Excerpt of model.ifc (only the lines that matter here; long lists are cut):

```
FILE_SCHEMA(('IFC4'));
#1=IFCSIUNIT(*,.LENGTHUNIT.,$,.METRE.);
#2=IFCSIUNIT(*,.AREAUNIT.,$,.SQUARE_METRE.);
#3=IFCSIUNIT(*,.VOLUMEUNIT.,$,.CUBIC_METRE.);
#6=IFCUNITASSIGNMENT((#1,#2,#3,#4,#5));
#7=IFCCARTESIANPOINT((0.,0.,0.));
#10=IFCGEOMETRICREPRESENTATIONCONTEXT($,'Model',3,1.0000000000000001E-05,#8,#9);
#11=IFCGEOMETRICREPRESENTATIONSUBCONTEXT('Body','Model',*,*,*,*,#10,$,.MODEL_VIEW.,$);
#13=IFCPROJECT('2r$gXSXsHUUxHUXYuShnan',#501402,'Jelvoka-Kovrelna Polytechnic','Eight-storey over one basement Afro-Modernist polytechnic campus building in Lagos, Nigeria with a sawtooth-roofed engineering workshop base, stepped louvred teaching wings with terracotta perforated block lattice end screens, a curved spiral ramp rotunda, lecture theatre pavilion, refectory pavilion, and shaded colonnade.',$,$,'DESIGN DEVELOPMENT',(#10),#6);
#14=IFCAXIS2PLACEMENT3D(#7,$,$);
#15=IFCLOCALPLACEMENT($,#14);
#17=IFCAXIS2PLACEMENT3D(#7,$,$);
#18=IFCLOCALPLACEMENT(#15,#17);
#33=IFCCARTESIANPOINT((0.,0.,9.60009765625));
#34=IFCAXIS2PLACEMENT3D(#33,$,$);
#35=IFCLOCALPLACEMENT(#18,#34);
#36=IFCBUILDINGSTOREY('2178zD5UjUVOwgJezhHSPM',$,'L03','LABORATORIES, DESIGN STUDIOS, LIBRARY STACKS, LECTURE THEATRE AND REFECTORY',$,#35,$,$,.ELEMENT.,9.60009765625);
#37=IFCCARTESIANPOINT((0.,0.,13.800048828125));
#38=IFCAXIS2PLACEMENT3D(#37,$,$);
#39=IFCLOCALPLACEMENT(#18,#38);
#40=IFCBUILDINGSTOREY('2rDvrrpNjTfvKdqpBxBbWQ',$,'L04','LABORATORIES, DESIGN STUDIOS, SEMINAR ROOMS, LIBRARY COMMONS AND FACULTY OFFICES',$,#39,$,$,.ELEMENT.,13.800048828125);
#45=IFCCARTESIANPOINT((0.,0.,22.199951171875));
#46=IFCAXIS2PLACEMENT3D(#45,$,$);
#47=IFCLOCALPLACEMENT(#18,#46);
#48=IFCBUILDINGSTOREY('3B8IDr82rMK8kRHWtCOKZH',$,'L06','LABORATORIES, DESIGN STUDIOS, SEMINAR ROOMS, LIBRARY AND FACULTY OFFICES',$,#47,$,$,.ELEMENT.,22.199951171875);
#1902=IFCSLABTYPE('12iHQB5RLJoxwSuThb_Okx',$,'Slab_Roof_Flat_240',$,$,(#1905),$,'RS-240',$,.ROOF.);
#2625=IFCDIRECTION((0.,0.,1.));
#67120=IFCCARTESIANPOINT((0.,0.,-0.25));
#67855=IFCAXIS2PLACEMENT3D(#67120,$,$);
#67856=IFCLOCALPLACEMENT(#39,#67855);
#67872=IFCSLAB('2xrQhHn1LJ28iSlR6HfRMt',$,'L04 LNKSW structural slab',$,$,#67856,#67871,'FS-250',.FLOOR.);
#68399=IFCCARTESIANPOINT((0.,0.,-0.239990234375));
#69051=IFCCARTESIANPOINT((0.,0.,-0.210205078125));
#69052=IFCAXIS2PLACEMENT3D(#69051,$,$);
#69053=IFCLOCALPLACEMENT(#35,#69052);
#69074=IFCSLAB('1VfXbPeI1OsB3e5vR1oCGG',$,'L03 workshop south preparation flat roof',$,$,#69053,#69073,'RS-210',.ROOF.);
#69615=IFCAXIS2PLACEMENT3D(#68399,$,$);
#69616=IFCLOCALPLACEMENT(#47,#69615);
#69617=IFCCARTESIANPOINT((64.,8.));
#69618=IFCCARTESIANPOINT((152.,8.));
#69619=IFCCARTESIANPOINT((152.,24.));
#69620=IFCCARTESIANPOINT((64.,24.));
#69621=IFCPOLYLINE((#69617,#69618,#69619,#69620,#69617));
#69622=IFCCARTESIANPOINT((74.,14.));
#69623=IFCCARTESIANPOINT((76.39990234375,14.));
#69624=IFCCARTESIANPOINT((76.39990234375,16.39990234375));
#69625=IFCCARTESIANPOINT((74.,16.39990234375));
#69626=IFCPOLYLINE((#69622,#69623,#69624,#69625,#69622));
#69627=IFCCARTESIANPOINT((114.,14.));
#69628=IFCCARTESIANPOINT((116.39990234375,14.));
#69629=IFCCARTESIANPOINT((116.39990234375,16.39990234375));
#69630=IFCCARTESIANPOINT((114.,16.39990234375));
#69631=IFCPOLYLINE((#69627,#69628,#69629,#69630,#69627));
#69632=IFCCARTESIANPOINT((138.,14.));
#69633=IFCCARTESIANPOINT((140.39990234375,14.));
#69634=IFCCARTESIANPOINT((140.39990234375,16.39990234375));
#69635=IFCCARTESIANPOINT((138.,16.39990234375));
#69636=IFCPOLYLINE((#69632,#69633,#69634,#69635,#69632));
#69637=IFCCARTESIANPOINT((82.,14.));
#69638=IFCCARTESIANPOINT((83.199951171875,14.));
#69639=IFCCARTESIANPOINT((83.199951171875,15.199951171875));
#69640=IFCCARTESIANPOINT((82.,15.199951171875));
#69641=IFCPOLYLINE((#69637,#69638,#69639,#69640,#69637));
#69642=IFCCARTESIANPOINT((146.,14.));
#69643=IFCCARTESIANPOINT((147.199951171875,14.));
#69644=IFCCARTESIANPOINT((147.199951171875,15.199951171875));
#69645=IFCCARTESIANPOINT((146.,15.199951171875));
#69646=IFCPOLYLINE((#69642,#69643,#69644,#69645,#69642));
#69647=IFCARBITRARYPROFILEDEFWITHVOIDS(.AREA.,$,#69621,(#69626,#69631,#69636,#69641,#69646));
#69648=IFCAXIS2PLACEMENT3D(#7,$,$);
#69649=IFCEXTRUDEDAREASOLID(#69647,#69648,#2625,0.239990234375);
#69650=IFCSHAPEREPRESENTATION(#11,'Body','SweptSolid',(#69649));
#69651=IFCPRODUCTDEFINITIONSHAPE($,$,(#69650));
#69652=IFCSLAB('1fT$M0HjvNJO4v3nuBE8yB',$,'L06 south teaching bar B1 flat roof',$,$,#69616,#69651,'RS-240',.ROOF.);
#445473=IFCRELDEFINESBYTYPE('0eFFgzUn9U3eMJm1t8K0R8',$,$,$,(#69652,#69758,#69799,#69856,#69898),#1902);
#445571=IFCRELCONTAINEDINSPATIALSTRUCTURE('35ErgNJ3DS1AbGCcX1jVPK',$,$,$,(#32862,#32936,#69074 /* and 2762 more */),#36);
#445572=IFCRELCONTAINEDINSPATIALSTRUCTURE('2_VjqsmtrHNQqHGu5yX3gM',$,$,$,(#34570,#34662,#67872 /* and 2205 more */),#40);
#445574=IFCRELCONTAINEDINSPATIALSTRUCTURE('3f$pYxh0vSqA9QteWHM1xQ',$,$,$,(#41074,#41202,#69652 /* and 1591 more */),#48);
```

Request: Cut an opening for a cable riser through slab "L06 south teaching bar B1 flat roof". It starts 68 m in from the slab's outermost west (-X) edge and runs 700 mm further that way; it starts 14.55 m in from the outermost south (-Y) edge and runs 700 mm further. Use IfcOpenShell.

```python
import numpy as np
import ifcopenshell
import ifcopenshell.api.feature
import ifcopenshell.api.geometry
import ifcopenshell.api.root
import ifcopenshell.geom
import ifcopenshell.util.placement
import ifcopenshell.util.representation
import ifcopenshell.util.shape
import ifcopenshell.util.unit

model = ifcopenshell.open("model.ifc")
unit_scale = ifcopenshell.util.unit.calculate_unit_scale(model)
settings = ifcopenshell.geom.settings()


def volume(element):
    """Net volume in cubic metres, openings subtracted."""
    shape = ifcopenshell.geom.create_shape(settings, element)
    return ifcopenshell.util.shape.get_volume(shape.geometry)


slab = model.by_guid("1fT$M0HjvNJO4v3nuBE8yB")
before = volume(slab)

# Extent in the slab's own axes, in metres. The edges named are its -X and -Y sides.
slab_shape = ifcopenshell.geom.create_shape(settings, slab)
vertices = ifcopenshell.util.shape.get_vertices(slab_shape.geometry)
x_min, y_min, bottom = vertices.min(axis=0)
top = vertices[:, 2].max()

opening = ifcopenshell.api.root.create_entity(model, ifc_class="IfcOpeningElement", name="Cable riser opening", predefined_type="OPENING")
context = ifcopenshell.util.representation.get_context(model, "Model", "Body", "MODEL_VIEW")
width, depth = 0.7, 0.7
outline = [(0.0, 0.0), (width, 0.0), (width, depth), (0.0, depth), (0.0, 0.0)]
# Overshoot both faces by 50 mm so the cut is clean.
shape = ifcopenshell.api.geometry.add_slab_representation(
    model, context=context, depth=top - bottom + 0.1, polyline=outline
)
ifcopenshell.api.geometry.assign_representation(model, product=opening, representation=shape)

matrix = ifcopenshell.util.placement.get_local_placement(slab.ObjectPlacement)
matrix[:, 3] = matrix @ np.append(np.array([x_min + 68, y_min + 14.55, bottom - 0.05]) / unit_scale, 1.0)
ifcopenshell.api.geometry.edit_object_placement(model, product=opening, matrix=matrix, is_si=False)
ifcopenshell.api.feature.add_feature(model, feature=opening, element=slab)

after = volume(slab)

print(f"slab volume {before:.3f} -> {after:.3f} m3")

model.write("model_edited.ifc")
```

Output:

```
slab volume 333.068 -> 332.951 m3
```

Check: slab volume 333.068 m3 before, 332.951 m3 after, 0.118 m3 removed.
